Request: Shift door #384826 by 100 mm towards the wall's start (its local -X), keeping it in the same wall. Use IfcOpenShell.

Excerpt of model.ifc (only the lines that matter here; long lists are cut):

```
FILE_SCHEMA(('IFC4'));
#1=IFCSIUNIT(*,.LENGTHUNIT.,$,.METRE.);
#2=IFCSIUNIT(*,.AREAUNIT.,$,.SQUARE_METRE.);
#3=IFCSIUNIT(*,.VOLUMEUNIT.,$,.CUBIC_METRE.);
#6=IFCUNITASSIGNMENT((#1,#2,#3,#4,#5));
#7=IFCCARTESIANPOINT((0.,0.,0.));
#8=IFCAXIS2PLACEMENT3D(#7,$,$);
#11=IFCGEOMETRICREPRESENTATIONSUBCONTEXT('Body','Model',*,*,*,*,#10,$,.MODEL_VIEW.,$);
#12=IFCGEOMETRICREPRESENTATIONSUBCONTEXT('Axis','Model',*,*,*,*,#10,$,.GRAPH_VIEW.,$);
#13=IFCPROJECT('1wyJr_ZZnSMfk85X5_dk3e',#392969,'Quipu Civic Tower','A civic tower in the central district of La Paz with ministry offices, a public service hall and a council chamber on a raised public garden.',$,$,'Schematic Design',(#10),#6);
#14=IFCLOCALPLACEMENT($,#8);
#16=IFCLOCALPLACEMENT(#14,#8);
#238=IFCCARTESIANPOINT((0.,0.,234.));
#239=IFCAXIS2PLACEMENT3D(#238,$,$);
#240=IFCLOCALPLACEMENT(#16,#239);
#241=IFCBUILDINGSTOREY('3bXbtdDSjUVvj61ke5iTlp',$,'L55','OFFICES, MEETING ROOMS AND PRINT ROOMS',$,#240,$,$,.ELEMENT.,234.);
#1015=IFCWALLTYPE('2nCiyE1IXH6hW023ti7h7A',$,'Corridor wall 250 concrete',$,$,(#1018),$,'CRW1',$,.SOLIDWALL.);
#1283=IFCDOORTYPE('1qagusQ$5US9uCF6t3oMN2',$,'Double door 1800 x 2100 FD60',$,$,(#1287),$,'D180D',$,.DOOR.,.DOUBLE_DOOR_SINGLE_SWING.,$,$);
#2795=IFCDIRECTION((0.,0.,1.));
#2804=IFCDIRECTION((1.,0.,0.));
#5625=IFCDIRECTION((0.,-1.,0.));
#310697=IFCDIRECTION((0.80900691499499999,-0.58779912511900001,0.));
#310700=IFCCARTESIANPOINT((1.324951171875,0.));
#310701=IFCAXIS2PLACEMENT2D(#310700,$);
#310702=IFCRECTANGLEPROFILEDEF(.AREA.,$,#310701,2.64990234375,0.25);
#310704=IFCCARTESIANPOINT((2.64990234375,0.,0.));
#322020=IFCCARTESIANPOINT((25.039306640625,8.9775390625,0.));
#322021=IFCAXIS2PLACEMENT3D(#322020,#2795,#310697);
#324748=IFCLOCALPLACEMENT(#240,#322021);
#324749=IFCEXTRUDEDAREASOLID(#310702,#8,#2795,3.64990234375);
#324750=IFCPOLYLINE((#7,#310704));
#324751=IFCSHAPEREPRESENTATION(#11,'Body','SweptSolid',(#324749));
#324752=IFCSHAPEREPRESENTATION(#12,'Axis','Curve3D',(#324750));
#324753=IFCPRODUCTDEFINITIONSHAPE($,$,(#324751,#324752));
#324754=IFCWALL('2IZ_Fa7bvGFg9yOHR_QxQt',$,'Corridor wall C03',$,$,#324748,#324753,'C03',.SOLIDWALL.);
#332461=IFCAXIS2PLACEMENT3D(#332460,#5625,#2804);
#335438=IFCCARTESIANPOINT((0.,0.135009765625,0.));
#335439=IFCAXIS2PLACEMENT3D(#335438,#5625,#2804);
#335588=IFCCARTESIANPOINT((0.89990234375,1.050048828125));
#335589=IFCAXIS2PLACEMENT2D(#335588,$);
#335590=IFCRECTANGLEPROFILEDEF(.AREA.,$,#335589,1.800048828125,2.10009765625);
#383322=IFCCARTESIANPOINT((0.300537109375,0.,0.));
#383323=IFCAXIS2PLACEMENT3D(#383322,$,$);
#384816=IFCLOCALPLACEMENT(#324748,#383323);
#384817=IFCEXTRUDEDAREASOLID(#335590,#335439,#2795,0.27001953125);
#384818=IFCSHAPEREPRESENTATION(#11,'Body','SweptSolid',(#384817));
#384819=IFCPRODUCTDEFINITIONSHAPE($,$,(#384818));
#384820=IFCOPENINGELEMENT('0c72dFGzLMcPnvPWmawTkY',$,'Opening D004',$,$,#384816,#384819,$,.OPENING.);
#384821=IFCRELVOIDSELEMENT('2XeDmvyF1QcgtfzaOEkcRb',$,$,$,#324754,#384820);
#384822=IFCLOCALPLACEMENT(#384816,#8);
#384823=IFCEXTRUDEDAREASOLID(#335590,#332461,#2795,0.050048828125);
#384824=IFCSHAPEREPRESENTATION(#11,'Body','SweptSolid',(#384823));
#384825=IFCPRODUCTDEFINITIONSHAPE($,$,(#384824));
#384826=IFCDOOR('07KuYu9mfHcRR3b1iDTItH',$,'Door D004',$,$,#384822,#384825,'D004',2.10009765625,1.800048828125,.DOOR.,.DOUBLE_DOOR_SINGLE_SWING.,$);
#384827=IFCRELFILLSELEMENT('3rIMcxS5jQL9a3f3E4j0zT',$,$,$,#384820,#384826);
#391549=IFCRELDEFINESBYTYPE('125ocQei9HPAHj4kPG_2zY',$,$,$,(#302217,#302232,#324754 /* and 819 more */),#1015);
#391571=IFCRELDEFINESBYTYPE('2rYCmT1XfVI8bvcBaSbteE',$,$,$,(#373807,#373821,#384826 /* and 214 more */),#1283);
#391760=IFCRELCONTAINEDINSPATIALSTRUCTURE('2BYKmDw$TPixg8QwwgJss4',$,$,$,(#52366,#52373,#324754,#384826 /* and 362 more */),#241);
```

```python
import ifcopenshell
import ifcopenshell.api.geometry
import ifcopenshell.util.placement

model = ifcopenshell.open("model.ifc")

door = model.by_guid("07KuYu9mfHcRR3b1iDTItH")
opening = door.FillsVoids[0].RelatingOpeningElement
wall = opening.VoidsElements[0].RelatingBuildingElement

wall_matrix = ifcopenshell.util.placement.get_local_placement(wall.ObjectPlacement)
shift = wall_matrix[:3, 0] * -0.1
before = ifcopenshell.util.placement.get_local_placement(door.ObjectPlacement)[:3, 3].copy()

# The door is placed relative to its opening, so it follows when the opening moves.
matrix = ifcopenshell.util.placement.get_local_placement(opening.ObjectPlacement)
matrix[:3, 3] += shift
ifcopenshell.api.geometry.edit_object_placement(
    model, product=opening, matrix=matrix, is_si=False, should_transform_children=True
)

after = ifcopenshell.util.placement.get_local_placement(door.ObjectPlacement)[:3, 3]
print("door moved by", (after - before).round(3) + 0.0)

model.write("model_v2.ifc")
```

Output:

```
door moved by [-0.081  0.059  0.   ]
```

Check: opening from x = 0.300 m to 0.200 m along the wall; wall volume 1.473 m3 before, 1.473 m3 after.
